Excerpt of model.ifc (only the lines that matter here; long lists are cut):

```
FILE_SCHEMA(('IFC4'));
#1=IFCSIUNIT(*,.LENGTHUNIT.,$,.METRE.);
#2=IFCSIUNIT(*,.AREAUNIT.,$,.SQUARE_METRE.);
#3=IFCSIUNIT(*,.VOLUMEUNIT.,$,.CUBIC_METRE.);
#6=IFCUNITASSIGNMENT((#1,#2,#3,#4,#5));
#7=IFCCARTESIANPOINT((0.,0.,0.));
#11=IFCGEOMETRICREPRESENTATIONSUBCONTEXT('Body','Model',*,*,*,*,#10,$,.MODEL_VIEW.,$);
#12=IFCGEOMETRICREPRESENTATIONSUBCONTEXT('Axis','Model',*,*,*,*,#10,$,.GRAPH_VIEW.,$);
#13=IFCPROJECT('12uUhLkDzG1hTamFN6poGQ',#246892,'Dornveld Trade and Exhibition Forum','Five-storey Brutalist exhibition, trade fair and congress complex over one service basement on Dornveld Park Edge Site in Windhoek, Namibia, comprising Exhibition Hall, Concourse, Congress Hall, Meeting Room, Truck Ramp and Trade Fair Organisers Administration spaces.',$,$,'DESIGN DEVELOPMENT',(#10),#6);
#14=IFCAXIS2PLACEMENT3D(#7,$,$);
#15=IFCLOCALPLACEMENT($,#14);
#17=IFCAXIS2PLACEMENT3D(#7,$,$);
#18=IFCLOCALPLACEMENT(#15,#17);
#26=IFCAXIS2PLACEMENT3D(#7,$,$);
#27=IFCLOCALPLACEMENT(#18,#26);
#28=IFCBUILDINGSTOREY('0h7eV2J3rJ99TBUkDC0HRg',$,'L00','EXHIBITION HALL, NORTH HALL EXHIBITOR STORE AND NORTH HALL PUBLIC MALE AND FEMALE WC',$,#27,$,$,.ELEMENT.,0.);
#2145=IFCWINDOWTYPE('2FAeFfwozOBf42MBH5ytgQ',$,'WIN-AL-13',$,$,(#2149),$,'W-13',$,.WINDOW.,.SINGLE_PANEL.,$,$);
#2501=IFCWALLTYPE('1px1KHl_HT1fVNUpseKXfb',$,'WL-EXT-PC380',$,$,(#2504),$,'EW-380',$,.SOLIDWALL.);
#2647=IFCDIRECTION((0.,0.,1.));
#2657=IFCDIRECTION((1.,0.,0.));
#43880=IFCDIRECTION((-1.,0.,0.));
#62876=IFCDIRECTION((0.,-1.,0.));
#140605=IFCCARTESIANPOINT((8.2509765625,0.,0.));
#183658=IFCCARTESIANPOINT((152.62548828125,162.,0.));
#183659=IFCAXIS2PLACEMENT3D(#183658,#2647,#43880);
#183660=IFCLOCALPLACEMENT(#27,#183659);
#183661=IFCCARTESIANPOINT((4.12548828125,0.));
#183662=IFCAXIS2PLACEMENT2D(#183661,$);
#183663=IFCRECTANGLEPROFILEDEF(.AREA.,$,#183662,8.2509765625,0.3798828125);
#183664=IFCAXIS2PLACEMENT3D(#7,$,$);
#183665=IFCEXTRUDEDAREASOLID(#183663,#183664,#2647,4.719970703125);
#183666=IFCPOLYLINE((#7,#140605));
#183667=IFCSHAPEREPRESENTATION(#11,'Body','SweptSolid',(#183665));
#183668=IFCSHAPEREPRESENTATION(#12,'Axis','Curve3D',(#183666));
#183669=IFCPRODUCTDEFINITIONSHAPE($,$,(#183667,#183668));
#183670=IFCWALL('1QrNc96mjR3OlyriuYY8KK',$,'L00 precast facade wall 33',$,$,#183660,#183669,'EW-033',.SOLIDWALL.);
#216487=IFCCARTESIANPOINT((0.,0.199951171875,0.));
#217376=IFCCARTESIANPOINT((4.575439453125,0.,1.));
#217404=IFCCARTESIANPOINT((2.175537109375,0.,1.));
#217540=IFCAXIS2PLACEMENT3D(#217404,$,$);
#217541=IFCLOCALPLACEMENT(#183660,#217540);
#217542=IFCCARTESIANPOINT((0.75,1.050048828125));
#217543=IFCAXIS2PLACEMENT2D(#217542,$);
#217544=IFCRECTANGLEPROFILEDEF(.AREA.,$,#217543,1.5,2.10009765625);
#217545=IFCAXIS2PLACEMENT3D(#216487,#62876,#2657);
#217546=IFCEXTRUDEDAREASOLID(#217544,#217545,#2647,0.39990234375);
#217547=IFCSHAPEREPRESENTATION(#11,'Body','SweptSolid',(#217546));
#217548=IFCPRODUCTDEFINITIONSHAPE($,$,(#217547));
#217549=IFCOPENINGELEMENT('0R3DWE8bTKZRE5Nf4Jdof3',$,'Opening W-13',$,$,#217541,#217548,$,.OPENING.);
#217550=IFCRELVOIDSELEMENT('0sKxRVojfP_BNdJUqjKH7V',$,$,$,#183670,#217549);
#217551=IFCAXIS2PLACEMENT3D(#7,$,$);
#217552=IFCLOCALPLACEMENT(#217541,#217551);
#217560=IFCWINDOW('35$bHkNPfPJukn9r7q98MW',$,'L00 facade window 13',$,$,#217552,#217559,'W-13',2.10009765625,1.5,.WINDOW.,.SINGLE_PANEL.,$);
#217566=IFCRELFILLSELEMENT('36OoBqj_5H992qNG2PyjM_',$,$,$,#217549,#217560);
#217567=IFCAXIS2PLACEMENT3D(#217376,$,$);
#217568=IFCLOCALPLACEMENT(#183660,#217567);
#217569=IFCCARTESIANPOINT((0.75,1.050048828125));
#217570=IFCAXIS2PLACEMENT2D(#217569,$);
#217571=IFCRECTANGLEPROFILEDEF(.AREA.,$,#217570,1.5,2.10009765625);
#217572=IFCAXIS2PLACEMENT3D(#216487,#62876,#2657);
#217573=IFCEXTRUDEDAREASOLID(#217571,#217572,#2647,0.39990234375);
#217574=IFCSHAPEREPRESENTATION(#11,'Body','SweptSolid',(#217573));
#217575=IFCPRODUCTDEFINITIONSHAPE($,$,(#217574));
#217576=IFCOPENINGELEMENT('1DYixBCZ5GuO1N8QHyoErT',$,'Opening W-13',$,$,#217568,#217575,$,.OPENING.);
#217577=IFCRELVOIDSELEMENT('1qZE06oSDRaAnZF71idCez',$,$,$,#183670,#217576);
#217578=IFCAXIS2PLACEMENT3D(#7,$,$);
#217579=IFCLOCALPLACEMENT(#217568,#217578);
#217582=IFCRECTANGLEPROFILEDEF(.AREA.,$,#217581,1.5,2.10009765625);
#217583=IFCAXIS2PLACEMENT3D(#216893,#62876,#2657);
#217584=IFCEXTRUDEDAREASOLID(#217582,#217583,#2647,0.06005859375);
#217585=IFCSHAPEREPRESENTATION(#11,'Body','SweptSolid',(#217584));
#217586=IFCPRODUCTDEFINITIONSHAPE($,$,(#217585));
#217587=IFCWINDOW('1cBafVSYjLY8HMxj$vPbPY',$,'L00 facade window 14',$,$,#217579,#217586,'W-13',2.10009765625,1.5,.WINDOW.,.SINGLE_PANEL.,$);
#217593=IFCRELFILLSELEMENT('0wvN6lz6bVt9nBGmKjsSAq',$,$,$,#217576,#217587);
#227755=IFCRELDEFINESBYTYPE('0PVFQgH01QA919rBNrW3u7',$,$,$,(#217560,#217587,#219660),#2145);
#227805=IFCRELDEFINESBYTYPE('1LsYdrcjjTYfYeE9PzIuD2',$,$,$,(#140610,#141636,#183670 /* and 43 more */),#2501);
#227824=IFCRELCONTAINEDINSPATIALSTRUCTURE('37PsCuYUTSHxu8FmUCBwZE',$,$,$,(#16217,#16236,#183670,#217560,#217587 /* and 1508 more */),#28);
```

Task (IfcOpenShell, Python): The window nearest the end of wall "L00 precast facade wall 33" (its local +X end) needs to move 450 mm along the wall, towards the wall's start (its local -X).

```python
import ifcopenshell
import ifcopenshell.api.geometry
import ifcopenshell.util.placement
import ifcopenshell.util.unit

model = ifcopenshell.open("model.ifc")
unit_scale = ifcopenshell.util.unit.calculate_unit_scale(model)

window = model.by_id(217587)
opening = window.FillsVoids[0].RelatingOpeningElement
wall = opening.VoidsElements[0].RelatingBuildingElement

wall_matrix = ifcopenshell.util.placement.get_local_placement(wall.ObjectPlacement)
shift = wall_matrix[:3, 0] * -0.45 / unit_scale
before = ifcopenshell.util.placement.get_local_placement(window.ObjectPlacement)[:3, 3].copy()

# The window is placed relative to its opening, so it follows when the opening moves.
matrix = ifcopenshell.util.placement.get_local_placement(opening.ObjectPlacement)
matrix[:3, 3] += shift
ifcopenshell.api.geometry.edit_object_placement(
    model, product=opening, matrix=matrix, is_si=False, should_transform_children=True
)

after = ifcopenshell.util.placement.get_local_placement(window.ObjectPlacement)[:3, 3]
print("window moved by", (after - before).round(3) + 0.0)

model.write("model_edited.ifc")
```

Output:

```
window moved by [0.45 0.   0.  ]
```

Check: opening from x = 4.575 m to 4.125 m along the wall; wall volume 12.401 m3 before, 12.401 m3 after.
